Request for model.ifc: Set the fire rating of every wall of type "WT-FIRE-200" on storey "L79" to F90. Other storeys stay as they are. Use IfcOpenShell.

First a look at what the model holds.

```python
import ifcopenshell
import ifcopenshell.util.element

model = ifcopenshell.open("model.ifc")
print(model.schema)
storey = next(s for s in model.by_type("IfcBuildingStorey") if s.Name == "L79")
walls = [e for e in ifcopenshell.util.element.get_decomposition(storey) if e.is_a("IfcWall")]
seen = {}
for e in walls:
    element_type = ifcopenshell.util.element.get_type(e)
    key = (element_type.Name if element_type != e and element_type else None, ifcopenshell.util.element.get_pset(e, "Pset_WallCommon", "FireRating"))
    seen[key] = seen.get(key, 0) + 1
for (name, value), count in sorted(seen.items(), key=str):
    print(count, "x", name, "|", value)
```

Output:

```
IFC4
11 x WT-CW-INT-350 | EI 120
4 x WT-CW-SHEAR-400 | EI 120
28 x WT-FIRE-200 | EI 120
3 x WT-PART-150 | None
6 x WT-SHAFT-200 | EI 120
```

```python
import ifcopenshell
import ifcopenshell.api.pset
import ifcopenshell.util.element

model = ifcopenshell.open("model.ifc")

storey = next(s for s in model.by_type("IfcBuildingStorey") if s.Name == "L79")
walls = [e for e in ifcopenshell.util.element.get_decomposition(storey) if e.is_a("IfcWall")]

count = 0
for e in walls:
    element_type = ifcopenshell.util.element.get_type(e)
    if element_type in (None, e) or element_type.Name != "WT-FIRE-200":
        continue
    found = ifcopenshell.util.element.get_pset(e, "Pset_WallCommon", should_inherit=False)
    if found:
        pset = model.by_id(found["id"])
        if len(ifcopenshell.util.element.get_elements_by_pset(pset)) > 1:
            pset = ifcopenshell.api.pset.unshare_pset(model, products=[e], pset=pset)[0]
    else:
        pset = ifcopenshell.api.pset.add_pset(model, product=e, name="Pset_WallCommon")
    ifcopenshell.api.pset.edit_pset(model, pset=pset, properties={"FireRating": "F90"})
    count += 1

print(count, "walls updated")

model.write("model_v2.ifc")
```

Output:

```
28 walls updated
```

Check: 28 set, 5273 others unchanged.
